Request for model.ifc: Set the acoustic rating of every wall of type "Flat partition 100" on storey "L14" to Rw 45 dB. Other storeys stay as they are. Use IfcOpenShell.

First a look at what the model holds.

```python
import ifcopenshell
import ifcopenshell.util.element

model = ifcopenshell.open("model.ifc")
print(model.schema)
storey = next(s for s in model.by_type("IfcBuildingStorey") if s.Name == "L14")
walls = [e for e in ifcopenshell.util.element.get_decomposition(storey) if e.is_a("IfcWall")]
seen = {}
for e in walls:
    element_type = ifcopenshell.util.element.get_type(e)
    key = (element_type.Name if element_type != e and element_type else None, ifcopenshell.util.element.get_pset(e, "Pset_WallCommon", "AcousticRating"))
    seen[key] = seen.get(key, 0) + 1
for (name, value), count in sorted(seen.items(), key=str):
    print(count, "x", name, "|", value)
```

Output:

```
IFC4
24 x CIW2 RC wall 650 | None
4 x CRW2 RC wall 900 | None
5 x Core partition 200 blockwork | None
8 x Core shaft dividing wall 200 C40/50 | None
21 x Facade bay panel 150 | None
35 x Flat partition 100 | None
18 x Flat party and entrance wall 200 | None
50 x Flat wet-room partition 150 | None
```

```python
import ifcopenshell
import ifcopenshell.api.pset
import ifcopenshell.util.element

model = ifcopenshell.open("model.ifc")

storey = next(s for s in model.by_type("IfcBuildingStorey") if s.Name == "L14")
walls = [e for e in ifcopenshell.util.element.get_decomposition(storey) if e.is_a("IfcWall")]

count = 0
for e in walls:
    element_type = ifcopenshell.util.element.get_type(e)
    if element_type in (None, e) or element_type.Name != "Flat partition 100":
        continue
    found = ifcopenshell.util.element.get_pset(e, "Pset_WallCommon", should_inherit=False)
    if found:
        pset = model.by_id(found["id"])
        if len(ifcopenshell.util.element.get_elements_by_pset(pset)) > 1:
            pset = ifcopenshell.api.pset.unshare_pset(model, products=[e], pset=pset)[0]
    else:
        pset = ifcopenshell.api.pset.add_pset(model, product=e, name="Pset_WallCommon")
    ifcopenshell.api.pset.edit_pset(model, pset=pset, properties={"AcousticRating": "Rw 45 dB"})
    count += 1

print(count, "walls updated")

model.write("model_edited.ifc")
```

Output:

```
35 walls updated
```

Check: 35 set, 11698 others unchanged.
